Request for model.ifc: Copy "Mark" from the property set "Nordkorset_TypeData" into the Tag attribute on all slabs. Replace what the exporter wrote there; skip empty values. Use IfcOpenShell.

First a look at what the model holds.

```python
import ifcopenshell
import ifcopenshell.util.element

model = ifcopenshell.open("model.ifc")
print(model.schema)
slabs = model.by_type("IfcSlab")
print(len(slabs), "slabs")
for e in slabs[:8]:
    source = ifcopenshell.util.element.get_pset(e, "Nordkorset_TypeData", "Mark")
    target = e.Tag
    print(e.id(), repr(source), repr(target), sep=" | ")
```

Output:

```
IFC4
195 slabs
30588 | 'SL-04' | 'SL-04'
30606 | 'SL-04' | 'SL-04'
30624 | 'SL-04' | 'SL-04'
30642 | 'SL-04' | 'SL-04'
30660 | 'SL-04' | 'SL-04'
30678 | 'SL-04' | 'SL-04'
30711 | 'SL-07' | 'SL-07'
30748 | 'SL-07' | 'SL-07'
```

```python
import ifcopenshell
import ifcopenshell.util.element

model = ifcopenshell.open("model.ifc")

count = 0
for e in model.by_type("IfcSlab"):
    value = ifcopenshell.util.element.get_pset(e, "Nordkorset_TypeData", "Mark")
    current = e.Tag
    if not value or not value.strip() or current == value:
        continue
    e.Tag = value
    count += 1

print(count, "slabs updated")

model.write("model_v2.ifc")
```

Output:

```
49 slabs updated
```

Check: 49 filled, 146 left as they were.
